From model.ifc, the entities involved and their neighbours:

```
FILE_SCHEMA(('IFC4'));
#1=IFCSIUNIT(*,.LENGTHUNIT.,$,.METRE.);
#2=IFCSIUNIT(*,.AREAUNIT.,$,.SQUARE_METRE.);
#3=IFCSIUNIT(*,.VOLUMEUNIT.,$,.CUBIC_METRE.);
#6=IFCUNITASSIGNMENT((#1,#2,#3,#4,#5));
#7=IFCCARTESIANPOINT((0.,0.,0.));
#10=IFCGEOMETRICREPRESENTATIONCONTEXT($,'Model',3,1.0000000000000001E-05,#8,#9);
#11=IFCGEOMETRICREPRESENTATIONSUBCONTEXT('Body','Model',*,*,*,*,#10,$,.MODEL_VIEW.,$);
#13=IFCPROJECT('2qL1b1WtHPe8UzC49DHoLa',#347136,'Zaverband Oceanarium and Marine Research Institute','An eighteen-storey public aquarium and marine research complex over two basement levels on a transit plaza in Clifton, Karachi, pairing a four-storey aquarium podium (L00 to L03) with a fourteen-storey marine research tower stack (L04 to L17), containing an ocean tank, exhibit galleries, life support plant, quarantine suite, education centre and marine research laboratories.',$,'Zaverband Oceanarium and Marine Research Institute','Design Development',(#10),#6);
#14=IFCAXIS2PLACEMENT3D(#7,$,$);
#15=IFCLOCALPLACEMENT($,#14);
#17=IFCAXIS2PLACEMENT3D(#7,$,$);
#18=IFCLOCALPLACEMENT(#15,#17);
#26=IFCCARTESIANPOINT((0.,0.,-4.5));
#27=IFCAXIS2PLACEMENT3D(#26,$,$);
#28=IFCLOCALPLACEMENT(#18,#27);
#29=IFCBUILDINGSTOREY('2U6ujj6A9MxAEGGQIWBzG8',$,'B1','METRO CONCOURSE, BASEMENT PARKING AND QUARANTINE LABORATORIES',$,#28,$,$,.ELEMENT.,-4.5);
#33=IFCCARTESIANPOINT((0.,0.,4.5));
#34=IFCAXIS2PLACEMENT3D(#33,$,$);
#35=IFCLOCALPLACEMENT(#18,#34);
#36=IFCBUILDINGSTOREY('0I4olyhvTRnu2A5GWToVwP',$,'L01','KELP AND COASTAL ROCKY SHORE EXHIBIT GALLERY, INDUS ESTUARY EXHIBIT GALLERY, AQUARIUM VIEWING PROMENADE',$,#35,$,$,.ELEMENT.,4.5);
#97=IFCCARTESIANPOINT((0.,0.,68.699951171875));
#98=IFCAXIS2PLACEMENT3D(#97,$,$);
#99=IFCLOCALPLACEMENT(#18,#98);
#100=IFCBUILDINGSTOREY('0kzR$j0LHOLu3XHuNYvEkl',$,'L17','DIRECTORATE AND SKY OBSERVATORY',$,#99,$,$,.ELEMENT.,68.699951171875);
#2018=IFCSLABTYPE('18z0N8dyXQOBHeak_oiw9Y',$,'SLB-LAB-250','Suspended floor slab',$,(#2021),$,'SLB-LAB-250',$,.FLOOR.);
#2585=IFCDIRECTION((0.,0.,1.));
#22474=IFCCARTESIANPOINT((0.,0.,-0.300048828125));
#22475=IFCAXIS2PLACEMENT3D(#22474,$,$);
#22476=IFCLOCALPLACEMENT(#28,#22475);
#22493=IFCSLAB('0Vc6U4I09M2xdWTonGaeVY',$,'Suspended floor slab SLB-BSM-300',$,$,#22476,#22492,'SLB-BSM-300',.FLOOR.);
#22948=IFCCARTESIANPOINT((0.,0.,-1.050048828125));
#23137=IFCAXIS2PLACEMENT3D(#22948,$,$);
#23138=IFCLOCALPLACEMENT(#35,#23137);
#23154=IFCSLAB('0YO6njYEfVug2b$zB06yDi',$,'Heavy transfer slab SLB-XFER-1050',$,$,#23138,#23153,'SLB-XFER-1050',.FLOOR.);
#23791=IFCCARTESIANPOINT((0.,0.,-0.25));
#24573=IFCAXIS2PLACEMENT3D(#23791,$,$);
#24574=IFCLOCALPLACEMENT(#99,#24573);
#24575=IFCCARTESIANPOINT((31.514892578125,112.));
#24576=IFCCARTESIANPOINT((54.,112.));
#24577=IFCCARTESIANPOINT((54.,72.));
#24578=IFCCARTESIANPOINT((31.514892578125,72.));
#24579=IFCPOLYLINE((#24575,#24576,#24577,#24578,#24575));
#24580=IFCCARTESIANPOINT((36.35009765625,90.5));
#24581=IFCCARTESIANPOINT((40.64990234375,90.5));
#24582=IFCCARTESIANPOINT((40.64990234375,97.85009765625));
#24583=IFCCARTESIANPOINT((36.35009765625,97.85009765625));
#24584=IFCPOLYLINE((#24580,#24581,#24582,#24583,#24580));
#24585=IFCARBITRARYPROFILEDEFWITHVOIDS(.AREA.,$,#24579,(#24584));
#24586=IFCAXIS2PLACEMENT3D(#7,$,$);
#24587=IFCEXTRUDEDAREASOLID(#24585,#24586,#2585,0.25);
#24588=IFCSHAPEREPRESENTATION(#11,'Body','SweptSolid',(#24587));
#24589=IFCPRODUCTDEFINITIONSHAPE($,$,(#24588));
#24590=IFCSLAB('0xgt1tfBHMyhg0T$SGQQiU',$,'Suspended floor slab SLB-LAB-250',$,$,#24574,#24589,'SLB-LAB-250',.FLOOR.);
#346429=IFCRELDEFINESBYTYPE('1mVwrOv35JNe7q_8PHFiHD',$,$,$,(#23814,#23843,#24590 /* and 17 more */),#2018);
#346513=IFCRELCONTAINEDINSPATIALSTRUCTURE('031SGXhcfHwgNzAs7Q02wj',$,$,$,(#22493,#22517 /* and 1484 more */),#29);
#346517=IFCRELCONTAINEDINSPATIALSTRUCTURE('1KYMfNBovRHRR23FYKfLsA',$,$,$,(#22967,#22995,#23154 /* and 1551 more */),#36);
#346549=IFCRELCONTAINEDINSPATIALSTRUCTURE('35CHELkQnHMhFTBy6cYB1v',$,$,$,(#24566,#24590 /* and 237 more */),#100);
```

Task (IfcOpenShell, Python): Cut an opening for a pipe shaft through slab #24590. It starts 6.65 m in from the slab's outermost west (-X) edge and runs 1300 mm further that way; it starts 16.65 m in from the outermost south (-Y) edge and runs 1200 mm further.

```python
import numpy as np
import ifcopenshell
import ifcopenshell.api.feature
import ifcopenshell.api.geometry
import ifcopenshell.api.root
import ifcopenshell.geom
import ifcopenshell.util.placement
import ifcopenshell.util.representation
import ifcopenshell.util.shape
import ifcopenshell.util.unit

model = ifcopenshell.open("model.ifc")
unit_scale = ifcopenshell.util.unit.calculate_unit_scale(model)
settings = ifcopenshell.geom.settings()


def volume(element):
    """Net volume in cubic metres, openings subtracted."""
    shape = ifcopenshell.geom.create_shape(settings, element)
    return ifcopenshell.util.shape.get_volume(shape.geometry)


slab = model.by_guid("0xgt1tfBHMyhg0T$SGQQiU")
before = volume(slab)

# Extent in the slab's own axes, in metres. The edges named are its -X and -Y sides.
slab_shape = ifcopenshell.geom.create_shape(settings, slab)
vertices = ifcopenshell.util.shape.get_vertices(slab_shape.geometry)
x_min, y_min, bottom = vertices.min(axis=0)
top = vertices[:, 2].max()

opening = ifcopenshell.api.root.create_entity(model, ifc_class="IfcOpeningElement", name="Pipe shaft opening", predefined_type="OPENING")
context = ifcopenshell.util.representation.get_context(model, "Model", "Body", "MODEL_VIEW")
width, depth = 1.3, 1.2
outline = [(0.0, 0.0), (width, 0.0), (width, depth), (0.0, depth), (0.0, 0.0)]
# Overshoot both faces by 50 mm so the cut is clean.
shape = ifcopenshell.api.geometry.add_slab_representation(
    model, context=context, depth=top - bottom + 0.1, polyline=outline
)
ifcopenshell.api.geometry.assign_representation(model, product=opening, representation=shape)

matrix = ifcopenshell.util.placement.get_local_placement(slab.ObjectPlacement)
matrix[:, 3] = matrix @ np.append(np.array([x_min + 6.65, y_min + 16.65, bottom - 0.05]) / unit_scale, 1.0)
ifcopenshell.api.geometry.edit_object_placement(model, product=opening, matrix=matrix, is_si=False)
ifcopenshell.api.feature.add_feature(model, feature=opening, element=slab)

after = volume(slab)

print(f"slab volume {before:.3f} -> {after:.3f} m3")

model.write("model_updated.ifc")
```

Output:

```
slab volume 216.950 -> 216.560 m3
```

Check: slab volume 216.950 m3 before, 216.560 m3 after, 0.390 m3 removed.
